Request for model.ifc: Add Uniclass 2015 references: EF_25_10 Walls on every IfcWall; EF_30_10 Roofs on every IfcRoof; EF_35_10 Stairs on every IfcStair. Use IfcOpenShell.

First a look at what the model holds.

```python
import ifcopenshell

model = ifcopenshell.open("model.ifc")
print(model.schema)
print("classifications:", [c.Name for c in model.by_type("IfcClassification")])
for ifc_class in ("IfcDoor", "IfcRoof", "IfcStair", "IfcWall", "IfcWindow"):
    print(ifc_class, len(model.by_type(ifc_class)))
```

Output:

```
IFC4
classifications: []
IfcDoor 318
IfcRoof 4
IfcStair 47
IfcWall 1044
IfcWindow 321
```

```python
import ifcopenshell
import ifcopenshell.api.classification

model = ifcopenshell.open("model.ifc")

system = ifcopenshell.api.classification.add_classification(model, classification="Uniclass 2015")

codes = {
    "IfcWall": ("EF_25_10", "Walls"),
    "IfcRoof": ("EF_30_10", "Roofs"),
    "IfcStair": ("EF_35_10", "Stairs"),
}
for ifc_class, (code, name) in codes.items():
    products = model.by_type(ifc_class)
    ifcopenshell.api.classification.add_reference(
        model, products=products, classification=system, identification=code, name=name
    )
    print(code, len(products))

model.write("model_edited.ifc")
```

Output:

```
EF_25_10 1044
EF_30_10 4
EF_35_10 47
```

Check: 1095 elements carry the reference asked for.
